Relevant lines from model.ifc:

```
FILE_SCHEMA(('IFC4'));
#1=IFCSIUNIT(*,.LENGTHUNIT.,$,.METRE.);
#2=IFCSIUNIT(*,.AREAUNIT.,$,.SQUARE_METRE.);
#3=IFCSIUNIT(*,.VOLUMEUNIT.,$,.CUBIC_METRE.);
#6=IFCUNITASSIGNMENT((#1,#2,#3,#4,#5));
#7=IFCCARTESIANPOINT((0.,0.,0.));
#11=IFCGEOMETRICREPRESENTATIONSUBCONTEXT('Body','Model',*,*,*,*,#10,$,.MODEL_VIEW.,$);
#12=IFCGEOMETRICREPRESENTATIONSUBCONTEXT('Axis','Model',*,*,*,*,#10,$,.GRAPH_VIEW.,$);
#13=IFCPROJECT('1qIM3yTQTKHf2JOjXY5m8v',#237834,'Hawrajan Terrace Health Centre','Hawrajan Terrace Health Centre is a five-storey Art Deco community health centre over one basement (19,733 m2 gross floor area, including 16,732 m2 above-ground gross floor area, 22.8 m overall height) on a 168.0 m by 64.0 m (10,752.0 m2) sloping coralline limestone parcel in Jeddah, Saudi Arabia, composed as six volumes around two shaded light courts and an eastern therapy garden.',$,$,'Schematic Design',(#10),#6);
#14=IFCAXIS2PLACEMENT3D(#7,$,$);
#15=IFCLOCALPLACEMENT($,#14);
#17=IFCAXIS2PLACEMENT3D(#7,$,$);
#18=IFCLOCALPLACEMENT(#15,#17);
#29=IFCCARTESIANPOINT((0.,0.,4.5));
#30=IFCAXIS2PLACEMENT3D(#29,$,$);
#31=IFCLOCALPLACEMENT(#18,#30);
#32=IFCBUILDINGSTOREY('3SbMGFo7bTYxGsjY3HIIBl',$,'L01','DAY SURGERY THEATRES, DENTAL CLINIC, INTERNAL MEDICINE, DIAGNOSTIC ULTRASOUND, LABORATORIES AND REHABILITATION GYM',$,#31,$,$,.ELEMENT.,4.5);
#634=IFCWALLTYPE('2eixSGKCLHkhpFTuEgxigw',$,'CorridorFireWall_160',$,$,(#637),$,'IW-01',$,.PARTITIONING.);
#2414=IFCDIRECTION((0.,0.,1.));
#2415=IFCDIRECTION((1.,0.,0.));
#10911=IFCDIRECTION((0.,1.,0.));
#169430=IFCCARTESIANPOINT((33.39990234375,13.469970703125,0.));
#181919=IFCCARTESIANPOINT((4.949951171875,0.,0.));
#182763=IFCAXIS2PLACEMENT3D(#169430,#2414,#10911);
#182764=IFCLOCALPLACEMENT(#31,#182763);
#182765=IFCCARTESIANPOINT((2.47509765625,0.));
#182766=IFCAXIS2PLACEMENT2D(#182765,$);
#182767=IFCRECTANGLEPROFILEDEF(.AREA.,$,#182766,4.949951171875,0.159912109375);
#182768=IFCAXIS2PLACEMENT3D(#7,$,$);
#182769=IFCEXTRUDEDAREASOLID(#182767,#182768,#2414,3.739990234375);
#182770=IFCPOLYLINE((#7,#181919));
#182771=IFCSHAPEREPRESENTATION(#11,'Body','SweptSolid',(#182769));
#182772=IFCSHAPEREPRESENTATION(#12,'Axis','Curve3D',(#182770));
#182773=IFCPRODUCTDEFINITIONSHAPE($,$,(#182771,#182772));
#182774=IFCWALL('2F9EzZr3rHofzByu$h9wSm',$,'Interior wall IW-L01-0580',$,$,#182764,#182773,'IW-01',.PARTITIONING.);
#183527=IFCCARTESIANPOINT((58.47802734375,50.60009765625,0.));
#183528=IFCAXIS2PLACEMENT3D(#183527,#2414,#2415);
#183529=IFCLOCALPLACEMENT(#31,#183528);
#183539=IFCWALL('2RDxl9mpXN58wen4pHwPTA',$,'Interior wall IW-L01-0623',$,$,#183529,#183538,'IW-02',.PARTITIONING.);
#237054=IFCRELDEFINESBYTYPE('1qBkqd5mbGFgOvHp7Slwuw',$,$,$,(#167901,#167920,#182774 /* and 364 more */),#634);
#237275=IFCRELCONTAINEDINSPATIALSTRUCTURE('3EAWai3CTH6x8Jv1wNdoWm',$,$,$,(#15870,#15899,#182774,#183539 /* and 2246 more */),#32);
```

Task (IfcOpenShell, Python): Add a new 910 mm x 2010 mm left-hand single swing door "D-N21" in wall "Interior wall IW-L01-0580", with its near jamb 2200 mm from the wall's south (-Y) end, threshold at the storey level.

```python
import numpy as np
import ifcopenshell
import ifcopenshell.api.feature
import ifcopenshell.api.geometry
import ifcopenshell.api.root
import ifcopenshell.api.spatial
import ifcopenshell.geom
import ifcopenshell.util.element
import ifcopenshell.util.placement
import ifcopenshell.util.representation
import ifcopenshell.util.shape
import ifcopenshell.util.unit

model = ifcopenshell.open("model.ifc")
unit_scale = ifcopenshell.util.unit.calculate_unit_scale(model)
settings = ifcopenshell.geom.settings()


def volume(element):
    """Net volume in cubic metres, openings subtracted."""
    shape = ifcopenshell.geom.create_shape(settings, element)
    return ifcopenshell.util.shape.get_volume(shape.geometry)


wall = model.by_guid("2F9EzZr3rHofzByu$h9wSm")
storey = ifcopenshell.util.element.get_container(wall, ifc_class="IfcBuildingStorey")
context = ifcopenshell.util.representation.get_context(model, "Model", "Body", "MODEL_VIEW")
before = volume(wall)

width, height, from_end, sill = 0.91, 2.01, 2.2, 0.0  # metres

# The wall runs along its own X axis, and the end named is its -X end.
wall_shape = ifcopenshell.geom.create_shape(settings, wall)
x, y, z = ifcopenshell.util.shape.get_vertices(wall_shape.geometry).T
start = x.min() + from_end
face, thickness = float(y.min()), float(y.max() - y.min())
wall_matrix = ifcopenshell.util.placement.get_local_placement(wall.ObjectPlacement)
level = ifcopenshell.util.placement.get_local_placement(storey.ObjectPlacement)[2, 3]


def in_wall(x, y):
    """Placement at x, y metres in the wall's axes, at sill height."""
    matrix = wall_matrix.copy()
    matrix[:, 3] = wall_matrix @ np.array([x / unit_scale, y / unit_scale, 0.0, 1.0])
    matrix[2, 3] = level + sill / unit_scale
    return matrix


# Opening: a box that overshoots both wall faces by 50 mm.
opening = ifcopenshell.api.root.create_entity(model, ifc_class="IfcOpeningElement", predefined_type="OPENING")
box = ifcopenshell.api.geometry.add_wall_representation(
    model, context=context, length=width, height=height, thickness=thickness + 0.1
)
ifcopenshell.api.geometry.assign_representation(model, product=opening, representation=box)
ifcopenshell.api.geometry.edit_object_placement(model, product=opening, matrix=in_wall(start, face - 0.05), is_si=False)
ifcopenshell.api.feature.add_feature(model, feature=opening, element=wall)

door = ifcopenshell.api.root.create_entity(model, ifc_class="IfcDoor", name="D-N21", predefined_type="DOOR")
door.OverallWidth, door.OverallHeight = width / unit_scale, height / unit_scale
door.OperationType = "SINGLE_SWING_LEFT"
body = ifcopenshell.api.geometry.add_door_representation(
    model,
    context=context,
    overall_width=door.OverallWidth,
    overall_height=door.OverallHeight,
    operation_type="SINGLE_SWING_LEFT",
    lining_properties={"LiningDepth": thickness / unit_scale, "ThresholdDepth": thickness / unit_scale},
)
ifcopenshell.api.geometry.assign_representation(model, product=door, representation=body)
ifcopenshell.api.spatial.assign_container(model, products=[door], relating_structure=storey)
ifcopenshell.api.feature.add_filling(model, opening=opening, element=door)

# The lining spans the wall, so the door starts at the wall face.
ifcopenshell.api.geometry.edit_object_placement(model, product=door, matrix=in_wall(start, face), is_si=False)

after = volume(wall)

print(f"wall volume {before:.3f} -> {after:.3f} m3")

model.write("model_v2.ifc")
```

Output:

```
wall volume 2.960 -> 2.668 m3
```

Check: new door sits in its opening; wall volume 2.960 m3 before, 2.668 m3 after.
